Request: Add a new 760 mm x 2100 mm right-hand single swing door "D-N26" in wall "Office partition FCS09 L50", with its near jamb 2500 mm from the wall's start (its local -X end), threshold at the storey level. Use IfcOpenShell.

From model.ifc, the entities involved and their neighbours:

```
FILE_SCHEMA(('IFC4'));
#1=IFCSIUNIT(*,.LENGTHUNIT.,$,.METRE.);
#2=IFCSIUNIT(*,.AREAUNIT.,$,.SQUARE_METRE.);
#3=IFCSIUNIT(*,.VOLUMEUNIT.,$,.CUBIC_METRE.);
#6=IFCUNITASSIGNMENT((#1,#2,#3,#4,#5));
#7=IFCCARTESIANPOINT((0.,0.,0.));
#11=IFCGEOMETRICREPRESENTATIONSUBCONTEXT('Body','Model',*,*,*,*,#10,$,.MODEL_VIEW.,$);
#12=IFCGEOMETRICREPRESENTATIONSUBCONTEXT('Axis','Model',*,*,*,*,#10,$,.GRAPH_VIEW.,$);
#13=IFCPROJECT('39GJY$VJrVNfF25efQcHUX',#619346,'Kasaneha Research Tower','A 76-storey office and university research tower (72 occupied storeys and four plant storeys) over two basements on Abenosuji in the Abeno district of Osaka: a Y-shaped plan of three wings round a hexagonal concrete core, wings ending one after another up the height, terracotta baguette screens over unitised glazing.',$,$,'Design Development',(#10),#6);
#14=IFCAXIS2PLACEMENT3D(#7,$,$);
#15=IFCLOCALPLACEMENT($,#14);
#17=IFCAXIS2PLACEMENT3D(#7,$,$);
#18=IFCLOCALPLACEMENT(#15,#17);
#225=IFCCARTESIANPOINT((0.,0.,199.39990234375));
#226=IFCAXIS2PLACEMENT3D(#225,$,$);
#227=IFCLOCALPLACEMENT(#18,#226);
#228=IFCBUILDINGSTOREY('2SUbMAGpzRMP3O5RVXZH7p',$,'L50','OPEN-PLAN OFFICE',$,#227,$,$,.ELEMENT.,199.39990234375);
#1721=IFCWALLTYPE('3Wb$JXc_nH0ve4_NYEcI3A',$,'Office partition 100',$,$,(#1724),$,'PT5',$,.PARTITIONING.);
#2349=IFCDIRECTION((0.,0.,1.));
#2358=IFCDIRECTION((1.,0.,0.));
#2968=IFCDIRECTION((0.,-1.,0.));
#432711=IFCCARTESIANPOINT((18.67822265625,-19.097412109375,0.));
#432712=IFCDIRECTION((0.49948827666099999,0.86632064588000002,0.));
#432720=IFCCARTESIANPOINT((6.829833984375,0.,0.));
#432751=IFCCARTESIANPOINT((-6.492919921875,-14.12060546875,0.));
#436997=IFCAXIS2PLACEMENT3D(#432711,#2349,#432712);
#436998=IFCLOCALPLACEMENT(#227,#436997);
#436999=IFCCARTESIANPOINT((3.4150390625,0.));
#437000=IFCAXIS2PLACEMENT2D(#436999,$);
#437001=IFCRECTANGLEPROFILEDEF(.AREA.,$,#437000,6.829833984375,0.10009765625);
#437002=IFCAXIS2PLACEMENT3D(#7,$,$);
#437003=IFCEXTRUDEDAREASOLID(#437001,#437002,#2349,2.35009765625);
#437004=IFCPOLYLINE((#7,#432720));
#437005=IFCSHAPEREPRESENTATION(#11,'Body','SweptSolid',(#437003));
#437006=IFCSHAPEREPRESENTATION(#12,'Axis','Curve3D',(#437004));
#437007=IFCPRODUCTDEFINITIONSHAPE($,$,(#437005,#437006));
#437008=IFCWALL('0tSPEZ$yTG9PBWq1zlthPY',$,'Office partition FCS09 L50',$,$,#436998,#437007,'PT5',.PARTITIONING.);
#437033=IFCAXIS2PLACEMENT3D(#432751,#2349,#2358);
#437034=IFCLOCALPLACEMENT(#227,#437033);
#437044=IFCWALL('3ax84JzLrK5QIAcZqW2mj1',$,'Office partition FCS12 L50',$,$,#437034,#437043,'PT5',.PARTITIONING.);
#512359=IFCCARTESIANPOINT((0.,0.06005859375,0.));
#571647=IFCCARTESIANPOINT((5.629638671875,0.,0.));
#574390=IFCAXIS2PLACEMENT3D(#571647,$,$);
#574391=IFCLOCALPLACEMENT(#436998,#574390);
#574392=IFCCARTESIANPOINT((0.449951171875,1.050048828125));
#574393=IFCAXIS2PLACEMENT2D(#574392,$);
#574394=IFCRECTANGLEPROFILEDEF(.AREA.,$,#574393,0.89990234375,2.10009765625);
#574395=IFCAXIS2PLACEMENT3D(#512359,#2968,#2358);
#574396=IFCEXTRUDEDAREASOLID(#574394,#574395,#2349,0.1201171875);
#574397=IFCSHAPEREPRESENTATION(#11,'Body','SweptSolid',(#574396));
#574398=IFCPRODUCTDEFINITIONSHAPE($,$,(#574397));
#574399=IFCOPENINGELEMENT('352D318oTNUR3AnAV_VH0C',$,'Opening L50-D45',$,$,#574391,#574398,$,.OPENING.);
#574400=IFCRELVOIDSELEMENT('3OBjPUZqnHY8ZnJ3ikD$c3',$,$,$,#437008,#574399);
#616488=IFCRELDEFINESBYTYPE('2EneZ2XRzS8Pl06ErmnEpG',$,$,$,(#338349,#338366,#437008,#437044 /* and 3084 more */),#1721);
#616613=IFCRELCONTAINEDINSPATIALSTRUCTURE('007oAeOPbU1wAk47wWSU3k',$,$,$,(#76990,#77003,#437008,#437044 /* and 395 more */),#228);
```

```python
import numpy as np
import ifcopenshell
import ifcopenshell.api.feature
import ifcopenshell.api.geometry
import ifcopenshell.api.root
import ifcopenshell.api.spatial
import ifcopenshell.geom
import ifcopenshell.util.element
import ifcopenshell.util.placement
import ifcopenshell.util.representation
import ifcopenshell.util.shape
import ifcopenshell.util.unit

model = ifcopenshell.open("model.ifc")
unit_scale = ifcopenshell.util.unit.calculate_unit_scale(model)
settings = ifcopenshell.geom.settings()


def volume(element):
    """Net volume in cubic metres, openings subtracted."""
    shape = ifcopenshell.geom.create_shape(settings, element)
    return ifcopenshell.util.shape.get_volume(shape.geometry)


wall = model.by_guid("0tSPEZ$yTG9PBWq1zlthPY")
storey = ifcopenshell.util.element.get_container(wall, ifc_class="IfcBuildingStorey")
context = ifcopenshell.util.representation.get_context(model, "Model", "Body", "MODEL_VIEW")
before = volume(wall)

width, height, from_end, sill = 0.76, 2.1, 2.5, 0.0  # metres

# The wall runs along its own X axis, and the end named is its -X end.
wall_shape = ifcopenshell.geom.create_shape(settings, wall)
x, y, z = ifcopenshell.util.shape.get_vertices(wall_shape.geometry).T
start = x.min() + from_end
face, thickness = float(y.min()), float(y.max() - y.min())
wall_matrix = ifcopenshell.util.placement.get_local_placement(wall.ObjectPlacement)
level = ifcopenshell.util.placement.get_local_placement(storey.ObjectPlacement)[2, 3]


def in_wall(x, y):
    """Placement at x, y metres in the wall's axes, at sill height."""
    matrix = wall_matrix.copy()
    matrix[:, 3] = wall_matrix @ np.array([x / unit_scale, y / unit_scale, 0.0, 1.0])
    matrix[2, 3] = level + sill / unit_scale
    return matrix


# Opening: a box that overshoots both wall faces by 50 mm.
opening = ifcopenshell.api.root.create_entity(model, ifc_class="IfcOpeningElement", predefined_type="OPENING")
box = ifcopenshell.api.geometry.add_wall_representation(
    model, context=context, length=width, height=height, thickness=thickness + 0.1
)
ifcopenshell.api.geometry.assign_representation(model, product=opening, representation=box)
ifcopenshell.api.geometry.edit_object_placement(model, product=opening, matrix=in_wall(start, face - 0.05), is_si=False)
ifcopenshell.api.feature.add_feature(model, feature=opening, element=wall)

door = ifcopenshell.api.root.create_entity(model, ifc_class="IfcDoor", name="D-N26", predefined_type="DOOR")
door.OverallWidth, door.OverallHeight = width / unit_scale, height / unit_scale
door.OperationType = "SINGLE_SWING_RIGHT"
body = ifcopenshell.api.geometry.add_door_representation(
    model,
    context=context,
    overall_width=door.OverallWidth,
    overall_height=door.OverallHeight,
    operation_type="SINGLE_SWING_RIGHT",
    lining_properties={"LiningDepth": thickness / unit_scale, "ThresholdDepth": thickness / unit_scale},
)
ifcopenshell.api.geometry.assign_representation(model, product=door, representation=body)
ifcopenshell.api.spatial.assign_container(model, products=[door], relating_structure=storey)
ifcopenshell.api.feature.add_filling(model, opening=opening, element=door)

# The lining spans the wall, so the door starts at the wall face.
ifcopenshell.api.geometry.edit_object_placement(model, product=door, matrix=in_wall(start, face), is_si=False)

after = volume(wall)

print(f"wall volume {before:.3f} -> {after:.3f} m3")

model.write("model_edited.ifc")
```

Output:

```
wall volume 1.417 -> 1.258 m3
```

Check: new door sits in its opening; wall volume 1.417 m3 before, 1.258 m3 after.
